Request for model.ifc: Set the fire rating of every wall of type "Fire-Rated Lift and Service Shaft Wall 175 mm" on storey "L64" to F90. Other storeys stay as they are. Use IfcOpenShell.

First a look at what the model holds.

```python
import ifcopenshell
import ifcopenshell.util.element

model = ifcopenshell.open("model.ifc")
print(model.schema)
storey = next(s for s in model.by_type("IfcBuildingStorey") if s.Name == "L64")
walls = [e for e in ifcopenshell.util.element.get_decomposition(storey) if e.is_a("IfcWall")]
seen = {}
for e in walls:
    element_type = ifcopenshell.util.element.get_type(e)
    key = (element_type.Name if element_type != e and element_type else None, ifcopenshell.util.element.get_pset(e, "Pset_WallCommon", "FireRating"))
    seen[key] = seen.get(key, 0) + 1
for (name, value), count in sorted(seen.items(), key=str):
    print(count, "x", name, "|", value)
```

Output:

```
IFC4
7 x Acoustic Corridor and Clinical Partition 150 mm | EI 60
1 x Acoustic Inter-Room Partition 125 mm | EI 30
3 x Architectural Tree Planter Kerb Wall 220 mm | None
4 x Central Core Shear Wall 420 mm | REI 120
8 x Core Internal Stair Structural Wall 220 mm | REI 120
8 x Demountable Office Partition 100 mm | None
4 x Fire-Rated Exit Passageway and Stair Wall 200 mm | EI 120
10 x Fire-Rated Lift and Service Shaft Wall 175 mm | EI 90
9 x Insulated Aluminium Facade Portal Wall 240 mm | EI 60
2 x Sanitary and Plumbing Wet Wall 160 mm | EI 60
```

```python
import ifcopenshell
import ifcopenshell.api.pset
import ifcopenshell.util.element

model = ifcopenshell.open("model.ifc")

storey = next(s for s in model.by_type("IfcBuildingStorey") if s.Name == "L64")
walls = [e for e in ifcopenshell.util.element.get_decomposition(storey) if e.is_a("IfcWall")]

count = 0
for e in walls:
    element_type = ifcopenshell.util.element.get_type(e)
    if element_type in (None, e) or element_type.Name != "Fire-Rated Lift and Service Shaft Wall 175 mm":
        continue
    found = ifcopenshell.util.element.get_pset(e, "Pset_WallCommon", should_inherit=False)
    if found:
        pset = model.by_id(found["id"])
        if len(ifcopenshell.util.element.get_elements_by_pset(pset)) > 1:
            pset = ifcopenshell.api.pset.unshare_pset(model, products=[e], pset=pset)[0]
    else:
        pset = ifcopenshell.api.pset.add_pset(model, product=e, name="Pset_WallCommon")
    ifcopenshell.api.pset.edit_pset(model, pset=pset, properties={"FireRating": "F90"})
    count += 1

print(count, "walls updated")

model.write("model_updated.ifc")
```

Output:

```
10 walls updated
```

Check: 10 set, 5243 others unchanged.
